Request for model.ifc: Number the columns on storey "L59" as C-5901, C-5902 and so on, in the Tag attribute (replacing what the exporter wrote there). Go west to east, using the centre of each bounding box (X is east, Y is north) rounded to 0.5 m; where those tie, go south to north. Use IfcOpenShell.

First a look at what the model holds.

```python
import ifcopenshell
import ifcopenshell.util.element
import ifcopenshell.util.placement

model = ifcopenshell.open("model.ifc")
print(model.schema)
storey = next(s for s in model.by_type("IfcBuildingStorey") if s.Name == "L59")
columns = [e for e in ifcopenshell.util.element.get_decomposition(storey) if e.is_a("IfcColumn")]
for e in sorted(columns, key=lambda e: e.id()):
    origin = ifcopenshell.util.placement.get_local_placement(e.ObjectPlacement)[:3, 3]
    print(e.id(), e.Tag, e.Name, origin.round(2) + 0.0, sep=" | ")
```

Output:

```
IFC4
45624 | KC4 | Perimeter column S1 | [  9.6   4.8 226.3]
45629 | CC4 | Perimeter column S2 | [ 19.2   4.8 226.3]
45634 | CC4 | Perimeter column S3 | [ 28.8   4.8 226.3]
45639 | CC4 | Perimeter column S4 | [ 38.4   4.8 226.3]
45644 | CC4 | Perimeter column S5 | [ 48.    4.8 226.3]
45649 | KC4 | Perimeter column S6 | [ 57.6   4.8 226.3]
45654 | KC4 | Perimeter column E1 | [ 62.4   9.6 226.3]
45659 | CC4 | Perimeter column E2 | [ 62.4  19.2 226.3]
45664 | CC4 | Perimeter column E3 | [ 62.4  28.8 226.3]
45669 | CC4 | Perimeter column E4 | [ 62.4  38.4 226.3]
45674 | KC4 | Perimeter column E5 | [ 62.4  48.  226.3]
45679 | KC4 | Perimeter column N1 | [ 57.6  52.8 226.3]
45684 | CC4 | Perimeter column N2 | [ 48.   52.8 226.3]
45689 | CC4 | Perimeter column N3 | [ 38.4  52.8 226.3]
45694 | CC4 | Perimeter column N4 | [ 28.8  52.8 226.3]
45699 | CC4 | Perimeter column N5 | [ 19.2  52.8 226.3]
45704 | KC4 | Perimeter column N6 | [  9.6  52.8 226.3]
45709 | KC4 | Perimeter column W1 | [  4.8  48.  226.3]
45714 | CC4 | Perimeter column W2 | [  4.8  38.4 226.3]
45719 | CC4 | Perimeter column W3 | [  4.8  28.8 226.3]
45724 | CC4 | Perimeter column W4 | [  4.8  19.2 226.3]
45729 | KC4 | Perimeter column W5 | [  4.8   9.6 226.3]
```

```python
import ifcopenshell
import ifcopenshell.geom
import ifcopenshell.util.element
import ifcopenshell.util.shape

model = ifcopenshell.open("model.ifc")
settings = ifcopenshell.geom.settings()
settings.set("use-world-coords", True)


def centre(element):
    shape = ifcopenshell.geom.create_shape(settings, element)
    return ifcopenshell.util.shape.get_bbox_centroid(shape.geometry)


storey = next(s for s in model.by_type("IfcBuildingStorey") if s.Name == "L59")
columns = [e for e in ifcopenshell.util.element.get_decomposition(storey) if e.is_a("IfcColumn")]

# Insertion points can sit at a corner or the storey origin, so sort by the geometry (in metres).
centres = {e: centre(e) for e in columns}
columns.sort(key=lambda e: (round(centres[e][0] / 0.5), centres[e][1]))

for i, e in enumerate(columns, start=1):
    number = f"C-59{i:02d}"
    e.Tag = number
    print(e.id(), number)

model.write("model-out.ifc")
```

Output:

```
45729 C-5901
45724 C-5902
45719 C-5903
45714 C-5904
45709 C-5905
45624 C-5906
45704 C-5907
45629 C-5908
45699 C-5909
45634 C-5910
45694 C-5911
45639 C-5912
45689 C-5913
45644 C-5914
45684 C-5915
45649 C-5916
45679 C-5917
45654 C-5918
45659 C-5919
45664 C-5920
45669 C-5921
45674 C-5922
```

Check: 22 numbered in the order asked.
